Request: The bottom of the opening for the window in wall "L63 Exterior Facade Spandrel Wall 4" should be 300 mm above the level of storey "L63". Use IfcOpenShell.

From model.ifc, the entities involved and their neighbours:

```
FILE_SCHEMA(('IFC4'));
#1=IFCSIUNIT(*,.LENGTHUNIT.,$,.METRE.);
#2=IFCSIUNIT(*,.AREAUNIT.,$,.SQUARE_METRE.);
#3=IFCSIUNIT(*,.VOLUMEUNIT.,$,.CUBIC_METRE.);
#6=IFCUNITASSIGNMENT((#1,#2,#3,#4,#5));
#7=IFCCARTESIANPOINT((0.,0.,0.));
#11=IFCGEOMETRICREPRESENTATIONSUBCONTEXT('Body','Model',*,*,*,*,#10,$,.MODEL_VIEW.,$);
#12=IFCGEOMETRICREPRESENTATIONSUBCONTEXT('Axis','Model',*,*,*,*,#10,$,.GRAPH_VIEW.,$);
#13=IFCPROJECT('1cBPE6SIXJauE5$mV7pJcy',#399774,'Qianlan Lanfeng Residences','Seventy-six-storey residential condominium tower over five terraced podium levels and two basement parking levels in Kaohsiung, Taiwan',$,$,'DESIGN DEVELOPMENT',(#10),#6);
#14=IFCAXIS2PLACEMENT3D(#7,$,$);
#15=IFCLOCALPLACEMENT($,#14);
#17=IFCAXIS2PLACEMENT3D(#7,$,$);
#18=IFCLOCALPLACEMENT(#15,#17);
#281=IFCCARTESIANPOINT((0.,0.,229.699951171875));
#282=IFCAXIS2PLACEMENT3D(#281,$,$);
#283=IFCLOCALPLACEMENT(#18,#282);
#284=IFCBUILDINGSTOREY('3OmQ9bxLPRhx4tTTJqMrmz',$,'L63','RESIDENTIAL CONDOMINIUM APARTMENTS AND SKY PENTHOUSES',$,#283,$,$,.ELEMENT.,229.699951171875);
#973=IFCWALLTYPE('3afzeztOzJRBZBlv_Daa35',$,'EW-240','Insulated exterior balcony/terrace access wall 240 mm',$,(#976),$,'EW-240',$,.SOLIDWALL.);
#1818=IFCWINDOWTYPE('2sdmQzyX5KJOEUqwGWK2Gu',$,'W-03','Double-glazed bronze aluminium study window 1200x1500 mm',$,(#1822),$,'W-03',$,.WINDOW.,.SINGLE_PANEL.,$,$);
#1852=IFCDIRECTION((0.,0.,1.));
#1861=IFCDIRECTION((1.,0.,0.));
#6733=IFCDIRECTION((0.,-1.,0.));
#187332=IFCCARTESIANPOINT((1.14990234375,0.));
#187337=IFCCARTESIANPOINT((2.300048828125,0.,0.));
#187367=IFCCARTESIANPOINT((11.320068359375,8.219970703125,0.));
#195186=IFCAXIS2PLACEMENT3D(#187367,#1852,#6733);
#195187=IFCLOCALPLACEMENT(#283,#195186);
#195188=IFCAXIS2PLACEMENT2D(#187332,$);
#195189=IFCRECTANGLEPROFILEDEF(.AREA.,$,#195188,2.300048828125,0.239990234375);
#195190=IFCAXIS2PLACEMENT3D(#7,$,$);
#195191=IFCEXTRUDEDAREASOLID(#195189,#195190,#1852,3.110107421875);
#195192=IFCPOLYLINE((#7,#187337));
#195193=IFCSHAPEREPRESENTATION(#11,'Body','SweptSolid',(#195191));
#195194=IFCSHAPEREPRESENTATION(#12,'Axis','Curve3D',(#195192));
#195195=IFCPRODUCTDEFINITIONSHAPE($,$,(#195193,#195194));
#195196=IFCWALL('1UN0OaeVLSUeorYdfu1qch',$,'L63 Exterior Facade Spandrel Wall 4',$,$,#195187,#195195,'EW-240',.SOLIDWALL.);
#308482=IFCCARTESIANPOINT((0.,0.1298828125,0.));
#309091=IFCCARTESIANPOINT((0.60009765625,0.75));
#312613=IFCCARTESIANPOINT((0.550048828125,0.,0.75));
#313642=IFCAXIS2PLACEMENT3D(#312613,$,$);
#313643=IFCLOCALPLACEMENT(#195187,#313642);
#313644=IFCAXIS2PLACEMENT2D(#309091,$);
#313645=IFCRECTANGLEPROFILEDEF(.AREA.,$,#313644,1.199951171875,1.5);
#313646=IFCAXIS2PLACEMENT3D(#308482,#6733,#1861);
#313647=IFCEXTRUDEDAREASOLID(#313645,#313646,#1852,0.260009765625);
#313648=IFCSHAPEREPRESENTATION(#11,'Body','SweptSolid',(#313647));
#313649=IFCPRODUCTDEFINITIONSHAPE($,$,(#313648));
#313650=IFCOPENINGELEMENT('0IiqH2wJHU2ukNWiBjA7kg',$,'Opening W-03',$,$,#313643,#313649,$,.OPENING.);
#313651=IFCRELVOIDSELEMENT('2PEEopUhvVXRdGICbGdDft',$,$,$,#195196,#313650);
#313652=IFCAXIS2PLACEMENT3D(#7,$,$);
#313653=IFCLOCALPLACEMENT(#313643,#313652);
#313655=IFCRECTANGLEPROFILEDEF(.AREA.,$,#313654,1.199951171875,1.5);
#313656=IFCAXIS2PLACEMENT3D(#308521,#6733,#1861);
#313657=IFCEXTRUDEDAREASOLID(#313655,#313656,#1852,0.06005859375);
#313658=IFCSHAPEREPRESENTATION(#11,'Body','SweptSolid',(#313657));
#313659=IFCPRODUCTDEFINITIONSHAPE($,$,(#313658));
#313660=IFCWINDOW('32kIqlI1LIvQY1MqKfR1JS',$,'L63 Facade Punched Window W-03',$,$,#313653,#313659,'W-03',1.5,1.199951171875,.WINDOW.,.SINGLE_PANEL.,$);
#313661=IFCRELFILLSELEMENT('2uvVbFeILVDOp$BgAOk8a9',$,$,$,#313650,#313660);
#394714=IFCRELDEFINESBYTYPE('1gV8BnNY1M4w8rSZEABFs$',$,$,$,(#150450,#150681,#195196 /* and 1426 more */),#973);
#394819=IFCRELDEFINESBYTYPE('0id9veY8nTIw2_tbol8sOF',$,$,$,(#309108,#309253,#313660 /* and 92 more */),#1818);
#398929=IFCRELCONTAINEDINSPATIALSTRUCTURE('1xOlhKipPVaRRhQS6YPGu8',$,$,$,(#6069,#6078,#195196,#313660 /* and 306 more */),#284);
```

```python
import numpy as np
import ifcopenshell
import ifcopenshell.api.geometry
import ifcopenshell.geom
import ifcopenshell.util.element
import ifcopenshell.util.placement
import ifcopenshell.util.shape
import ifcopenshell.util.unit

model = ifcopenshell.open("model.ifc")
unit_scale = ifcopenshell.util.unit.calculate_unit_scale(model)

window = model.by_guid("32kIqlI1LIvQY1MqKfR1JS")
opening = window.FillsVoids[0].RelatingOpeningElement
storey = ifcopenshell.util.element.get_container(window, ifc_class="IfcBuildingStorey")
level = ifcopenshell.util.placement.get_local_placement(storey.ObjectPlacement)[2, 3]

# The opening's origin need not be at the sill, so measure its lowest point.
shape = ifcopenshell.geom.create_shape(ifcopenshell.geom.settings(), opening)
bottom = ifcopenshell.util.shape.get_shape_bottom_elevation(shape, shape.geometry) / unit_scale
dz = level + 0.3 / unit_scale - bottom

shift = np.array([0.0, 0.0, dz])
# The window is placed relative to its opening, so it follows when the opening moves.
matrix = ifcopenshell.util.placement.get_local_placement(opening.ObjectPlacement)
matrix[:3, 3] += shift
ifcopenshell.api.geometry.edit_object_placement(
    model, product=opening, matrix=matrix, is_si=False, should_transform_children=True
)

print(f"moved by {dz * unit_scale:+.3f} m")

model.write("model-out.ifc")
```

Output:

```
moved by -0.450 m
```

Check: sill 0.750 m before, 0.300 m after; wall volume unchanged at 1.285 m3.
